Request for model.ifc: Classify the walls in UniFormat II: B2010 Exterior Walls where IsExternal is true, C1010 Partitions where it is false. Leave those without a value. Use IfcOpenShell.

First a look at what the model holds.

```python
import ifcopenshell
import ifcopenshell.util.element

model = ifcopenshell.open("model.ifc")
print(model.schema)
print("classifications:", [c.Name for c in model.by_type("IfcClassification")])
values = [ifcopenshell.util.element.get_pset(e, "Pset_WallCommon", "IsExternal") for e in model.by_type("IfcWall")]
for value in (True, False, None):
    print("IsExternal", value, values.count(value))
```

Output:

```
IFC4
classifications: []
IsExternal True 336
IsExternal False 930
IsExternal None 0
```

```python
import ifcopenshell
import ifcopenshell.api.classification
import ifcopenshell.util.element

model = ifcopenshell.open("model.ifc")

system = ifcopenshell.api.classification.add_classification(model, classification="UniFormat II")

walls = model.by_type("IfcWall")
external = {e: ifcopenshell.util.element.get_pset(e, "Pset_WallCommon", "IsExternal") for e in walls}
for flag, code, name in ((True, "B2010", "Exterior Walls"), (False, "C1010", "Partitions")):
    products = [e for e in walls if external[e] is flag]
    ifcopenshell.api.classification.add_reference(
        model, products=products, classification=system, identification=code, name=name
    )
    print(code, len(products))

model.write("model_updated.ifc")
```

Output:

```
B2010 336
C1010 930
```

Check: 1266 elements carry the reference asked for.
